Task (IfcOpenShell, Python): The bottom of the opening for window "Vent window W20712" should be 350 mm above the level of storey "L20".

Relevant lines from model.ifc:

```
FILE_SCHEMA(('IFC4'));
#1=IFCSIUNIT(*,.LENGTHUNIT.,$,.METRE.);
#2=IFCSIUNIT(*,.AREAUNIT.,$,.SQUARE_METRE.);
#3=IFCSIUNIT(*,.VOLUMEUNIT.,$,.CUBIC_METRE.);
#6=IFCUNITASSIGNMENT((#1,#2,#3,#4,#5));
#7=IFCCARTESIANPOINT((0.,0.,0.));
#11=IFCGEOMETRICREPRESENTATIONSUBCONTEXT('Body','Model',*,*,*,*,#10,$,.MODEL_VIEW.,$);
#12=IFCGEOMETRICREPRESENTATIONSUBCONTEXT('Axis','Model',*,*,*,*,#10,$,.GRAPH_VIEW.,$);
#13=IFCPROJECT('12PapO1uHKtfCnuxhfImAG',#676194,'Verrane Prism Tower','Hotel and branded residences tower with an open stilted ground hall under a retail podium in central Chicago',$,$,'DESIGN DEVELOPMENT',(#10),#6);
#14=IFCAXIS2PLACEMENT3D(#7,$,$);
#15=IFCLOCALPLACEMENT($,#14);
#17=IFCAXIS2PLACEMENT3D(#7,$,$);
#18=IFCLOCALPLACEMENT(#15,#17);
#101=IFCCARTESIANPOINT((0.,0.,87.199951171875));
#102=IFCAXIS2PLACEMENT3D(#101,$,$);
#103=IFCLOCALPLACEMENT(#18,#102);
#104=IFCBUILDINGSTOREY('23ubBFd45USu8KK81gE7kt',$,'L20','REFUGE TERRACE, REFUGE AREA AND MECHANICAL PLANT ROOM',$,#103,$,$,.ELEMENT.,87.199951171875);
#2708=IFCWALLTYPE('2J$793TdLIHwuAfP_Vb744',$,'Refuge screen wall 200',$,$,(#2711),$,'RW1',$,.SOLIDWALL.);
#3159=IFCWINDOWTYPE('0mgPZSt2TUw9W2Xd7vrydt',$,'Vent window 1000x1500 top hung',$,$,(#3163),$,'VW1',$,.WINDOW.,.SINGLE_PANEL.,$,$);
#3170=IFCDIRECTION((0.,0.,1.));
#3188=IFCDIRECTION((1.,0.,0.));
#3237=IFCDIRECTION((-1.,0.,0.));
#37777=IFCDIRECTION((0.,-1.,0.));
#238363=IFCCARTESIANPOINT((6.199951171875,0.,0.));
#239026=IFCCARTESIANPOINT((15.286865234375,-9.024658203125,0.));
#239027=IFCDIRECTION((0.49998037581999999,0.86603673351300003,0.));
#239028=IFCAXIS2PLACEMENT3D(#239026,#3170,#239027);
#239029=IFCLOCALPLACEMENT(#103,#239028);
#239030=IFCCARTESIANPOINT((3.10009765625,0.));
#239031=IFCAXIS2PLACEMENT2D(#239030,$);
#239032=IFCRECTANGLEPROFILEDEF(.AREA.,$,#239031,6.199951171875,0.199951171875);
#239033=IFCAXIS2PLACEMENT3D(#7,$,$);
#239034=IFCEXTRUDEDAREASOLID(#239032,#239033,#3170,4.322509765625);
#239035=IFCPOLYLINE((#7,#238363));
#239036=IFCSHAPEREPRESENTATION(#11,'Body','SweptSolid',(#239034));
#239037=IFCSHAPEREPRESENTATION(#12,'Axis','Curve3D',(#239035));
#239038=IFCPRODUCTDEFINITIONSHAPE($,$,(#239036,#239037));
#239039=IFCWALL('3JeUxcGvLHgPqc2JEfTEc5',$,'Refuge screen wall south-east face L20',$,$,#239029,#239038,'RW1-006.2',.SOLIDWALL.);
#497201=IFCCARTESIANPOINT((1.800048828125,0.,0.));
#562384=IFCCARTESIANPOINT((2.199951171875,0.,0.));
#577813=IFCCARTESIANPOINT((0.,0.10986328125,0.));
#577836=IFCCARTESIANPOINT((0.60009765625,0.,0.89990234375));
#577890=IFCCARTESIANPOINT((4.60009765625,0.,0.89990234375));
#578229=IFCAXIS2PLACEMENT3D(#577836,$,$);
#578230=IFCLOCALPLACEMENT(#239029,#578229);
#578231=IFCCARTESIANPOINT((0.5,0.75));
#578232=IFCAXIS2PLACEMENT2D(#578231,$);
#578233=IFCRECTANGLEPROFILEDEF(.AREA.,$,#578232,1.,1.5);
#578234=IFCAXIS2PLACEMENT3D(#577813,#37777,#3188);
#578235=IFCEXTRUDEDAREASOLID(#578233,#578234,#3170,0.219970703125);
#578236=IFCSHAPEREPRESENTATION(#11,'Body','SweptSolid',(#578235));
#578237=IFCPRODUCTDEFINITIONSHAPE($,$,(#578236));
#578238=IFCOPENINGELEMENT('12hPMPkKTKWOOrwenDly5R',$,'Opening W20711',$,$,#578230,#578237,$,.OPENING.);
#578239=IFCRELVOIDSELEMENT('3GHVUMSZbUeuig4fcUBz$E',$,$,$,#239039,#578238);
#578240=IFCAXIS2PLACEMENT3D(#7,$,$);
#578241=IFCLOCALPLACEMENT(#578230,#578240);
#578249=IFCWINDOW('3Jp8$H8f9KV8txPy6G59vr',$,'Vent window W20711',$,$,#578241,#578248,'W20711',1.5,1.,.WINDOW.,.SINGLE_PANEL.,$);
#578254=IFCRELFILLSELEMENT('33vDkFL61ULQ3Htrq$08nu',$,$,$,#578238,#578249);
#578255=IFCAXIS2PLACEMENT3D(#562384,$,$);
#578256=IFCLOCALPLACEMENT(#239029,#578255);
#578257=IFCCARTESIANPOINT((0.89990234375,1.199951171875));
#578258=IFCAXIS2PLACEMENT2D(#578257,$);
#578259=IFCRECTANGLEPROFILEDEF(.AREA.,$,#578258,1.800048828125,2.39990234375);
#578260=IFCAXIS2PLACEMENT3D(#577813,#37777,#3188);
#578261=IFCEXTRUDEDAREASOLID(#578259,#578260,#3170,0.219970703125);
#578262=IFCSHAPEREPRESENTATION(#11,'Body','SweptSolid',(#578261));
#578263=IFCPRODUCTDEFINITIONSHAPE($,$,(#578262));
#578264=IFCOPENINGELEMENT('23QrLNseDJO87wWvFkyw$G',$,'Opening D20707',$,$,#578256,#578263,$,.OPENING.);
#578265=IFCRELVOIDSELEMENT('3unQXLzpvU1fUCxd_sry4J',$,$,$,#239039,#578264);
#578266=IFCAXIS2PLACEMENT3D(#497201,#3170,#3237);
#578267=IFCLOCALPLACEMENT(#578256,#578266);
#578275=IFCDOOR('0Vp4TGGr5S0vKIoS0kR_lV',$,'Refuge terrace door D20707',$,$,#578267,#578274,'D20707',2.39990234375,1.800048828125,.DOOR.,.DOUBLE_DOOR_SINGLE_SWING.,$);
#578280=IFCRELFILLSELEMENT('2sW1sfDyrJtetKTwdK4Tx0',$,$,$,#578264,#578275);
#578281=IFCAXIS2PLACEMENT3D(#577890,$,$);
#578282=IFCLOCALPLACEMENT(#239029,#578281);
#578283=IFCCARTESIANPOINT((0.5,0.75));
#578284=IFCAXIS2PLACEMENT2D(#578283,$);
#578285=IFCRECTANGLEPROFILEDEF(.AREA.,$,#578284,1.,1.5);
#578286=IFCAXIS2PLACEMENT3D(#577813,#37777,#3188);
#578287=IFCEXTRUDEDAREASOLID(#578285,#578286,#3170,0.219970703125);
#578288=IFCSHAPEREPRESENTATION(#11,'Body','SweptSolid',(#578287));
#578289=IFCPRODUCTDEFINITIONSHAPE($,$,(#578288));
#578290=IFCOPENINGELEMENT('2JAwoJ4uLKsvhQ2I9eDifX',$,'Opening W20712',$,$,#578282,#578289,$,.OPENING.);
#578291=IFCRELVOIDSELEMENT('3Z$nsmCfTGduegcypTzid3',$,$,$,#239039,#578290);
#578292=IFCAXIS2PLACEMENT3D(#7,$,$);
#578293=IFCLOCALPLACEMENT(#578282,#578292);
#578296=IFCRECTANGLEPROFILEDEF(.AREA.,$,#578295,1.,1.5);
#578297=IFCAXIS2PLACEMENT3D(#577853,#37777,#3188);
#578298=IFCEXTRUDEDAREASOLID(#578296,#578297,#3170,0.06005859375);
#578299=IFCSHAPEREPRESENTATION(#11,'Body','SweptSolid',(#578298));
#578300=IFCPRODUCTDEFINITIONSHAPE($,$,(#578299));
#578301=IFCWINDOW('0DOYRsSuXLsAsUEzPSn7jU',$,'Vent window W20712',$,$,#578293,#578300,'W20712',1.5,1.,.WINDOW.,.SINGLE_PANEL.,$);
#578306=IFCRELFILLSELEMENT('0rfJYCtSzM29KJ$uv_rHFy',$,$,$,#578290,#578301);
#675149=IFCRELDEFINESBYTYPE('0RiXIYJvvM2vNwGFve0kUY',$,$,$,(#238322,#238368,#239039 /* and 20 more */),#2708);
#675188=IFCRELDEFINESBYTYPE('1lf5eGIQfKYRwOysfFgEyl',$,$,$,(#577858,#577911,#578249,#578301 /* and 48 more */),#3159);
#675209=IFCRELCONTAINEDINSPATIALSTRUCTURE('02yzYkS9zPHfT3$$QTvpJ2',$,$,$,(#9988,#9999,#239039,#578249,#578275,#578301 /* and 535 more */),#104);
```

```python
import numpy as np
import ifcopenshell
import ifcopenshell.api.geometry
import ifcopenshell.geom
import ifcopenshell.util.element
import ifcopenshell.util.placement
import ifcopenshell.util.shape
import ifcopenshell.util.unit

model = ifcopenshell.open("model.ifc")
unit_scale = ifcopenshell.util.unit.calculate_unit_scale(model)

window = model.by_guid("0DOYRsSuXLsAsUEzPSn7jU")
opening = window.FillsVoids[0].RelatingOpeningElement
storey = ifcopenshell.util.element.get_container(window, ifc_class="IfcBuildingStorey")
level = ifcopenshell.util.placement.get_local_placement(storey.ObjectPlacement)[2, 3]

# The opening's origin need not be at the sill, so measure its lowest point.
shape = ifcopenshell.geom.create_shape(ifcopenshell.geom.settings(), opening)
bottom = ifcopenshell.util.shape.get_shape_bottom_elevation(shape, shape.geometry) / unit_scale
dz = level + 0.35 / unit_scale - bottom

shift = np.array([0.0, 0.0, dz])
# The window is placed relative to its opening, so it follows when the opening moves.
matrix = ifcopenshell.util.placement.get_local_placement(opening.ObjectPlacement)
matrix[:3, 3] += shift
ifcopenshell.api.geometry.edit_object_placement(
    model, product=opening, matrix=matrix, is_si=False, should_transform_children=True
)

print(f"moved by {dz * unit_scale:+.3f} m")

model.write("model_rev.ifc")
```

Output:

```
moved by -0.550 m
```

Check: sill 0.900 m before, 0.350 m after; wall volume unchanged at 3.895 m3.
